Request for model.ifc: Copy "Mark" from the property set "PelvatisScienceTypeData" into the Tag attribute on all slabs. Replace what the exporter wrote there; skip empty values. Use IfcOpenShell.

First a look at what the model holds.

```python
import ifcopenshell
import ifcopenshell.util.element

model = ifcopenshell.open("model.ifc")
print(model.schema)
slabs = model.by_type("IfcSlab")
print(len(slabs), "slabs")
for e in slabs[:8]:
    source = ifcopenshell.util.element.get_pset(e, "PelvatisScienceTypeData", "Mark")
    target = e.Tag
    print(e.id(), repr(source), repr(target), sep=" | ")
```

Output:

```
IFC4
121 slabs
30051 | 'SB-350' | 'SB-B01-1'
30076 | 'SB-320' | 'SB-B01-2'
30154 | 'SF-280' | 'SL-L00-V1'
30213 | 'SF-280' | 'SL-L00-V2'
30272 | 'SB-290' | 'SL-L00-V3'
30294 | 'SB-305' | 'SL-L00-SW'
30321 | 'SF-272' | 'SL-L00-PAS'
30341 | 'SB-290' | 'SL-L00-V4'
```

```python
import ifcopenshell
import ifcopenshell.util.element

model = ifcopenshell.open("model.ifc")

count = 0
for e in model.by_type("IfcSlab"):
    value = ifcopenshell.util.element.get_pset(e, "PelvatisScienceTypeData", "Mark")
    current = e.Tag
    if not value or not value.strip() or current == value:
        continue
    e.Tag = value
    count += 1

print(count, "slabs updated")

model.write("model_v2.ifc")
```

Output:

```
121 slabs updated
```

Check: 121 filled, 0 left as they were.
